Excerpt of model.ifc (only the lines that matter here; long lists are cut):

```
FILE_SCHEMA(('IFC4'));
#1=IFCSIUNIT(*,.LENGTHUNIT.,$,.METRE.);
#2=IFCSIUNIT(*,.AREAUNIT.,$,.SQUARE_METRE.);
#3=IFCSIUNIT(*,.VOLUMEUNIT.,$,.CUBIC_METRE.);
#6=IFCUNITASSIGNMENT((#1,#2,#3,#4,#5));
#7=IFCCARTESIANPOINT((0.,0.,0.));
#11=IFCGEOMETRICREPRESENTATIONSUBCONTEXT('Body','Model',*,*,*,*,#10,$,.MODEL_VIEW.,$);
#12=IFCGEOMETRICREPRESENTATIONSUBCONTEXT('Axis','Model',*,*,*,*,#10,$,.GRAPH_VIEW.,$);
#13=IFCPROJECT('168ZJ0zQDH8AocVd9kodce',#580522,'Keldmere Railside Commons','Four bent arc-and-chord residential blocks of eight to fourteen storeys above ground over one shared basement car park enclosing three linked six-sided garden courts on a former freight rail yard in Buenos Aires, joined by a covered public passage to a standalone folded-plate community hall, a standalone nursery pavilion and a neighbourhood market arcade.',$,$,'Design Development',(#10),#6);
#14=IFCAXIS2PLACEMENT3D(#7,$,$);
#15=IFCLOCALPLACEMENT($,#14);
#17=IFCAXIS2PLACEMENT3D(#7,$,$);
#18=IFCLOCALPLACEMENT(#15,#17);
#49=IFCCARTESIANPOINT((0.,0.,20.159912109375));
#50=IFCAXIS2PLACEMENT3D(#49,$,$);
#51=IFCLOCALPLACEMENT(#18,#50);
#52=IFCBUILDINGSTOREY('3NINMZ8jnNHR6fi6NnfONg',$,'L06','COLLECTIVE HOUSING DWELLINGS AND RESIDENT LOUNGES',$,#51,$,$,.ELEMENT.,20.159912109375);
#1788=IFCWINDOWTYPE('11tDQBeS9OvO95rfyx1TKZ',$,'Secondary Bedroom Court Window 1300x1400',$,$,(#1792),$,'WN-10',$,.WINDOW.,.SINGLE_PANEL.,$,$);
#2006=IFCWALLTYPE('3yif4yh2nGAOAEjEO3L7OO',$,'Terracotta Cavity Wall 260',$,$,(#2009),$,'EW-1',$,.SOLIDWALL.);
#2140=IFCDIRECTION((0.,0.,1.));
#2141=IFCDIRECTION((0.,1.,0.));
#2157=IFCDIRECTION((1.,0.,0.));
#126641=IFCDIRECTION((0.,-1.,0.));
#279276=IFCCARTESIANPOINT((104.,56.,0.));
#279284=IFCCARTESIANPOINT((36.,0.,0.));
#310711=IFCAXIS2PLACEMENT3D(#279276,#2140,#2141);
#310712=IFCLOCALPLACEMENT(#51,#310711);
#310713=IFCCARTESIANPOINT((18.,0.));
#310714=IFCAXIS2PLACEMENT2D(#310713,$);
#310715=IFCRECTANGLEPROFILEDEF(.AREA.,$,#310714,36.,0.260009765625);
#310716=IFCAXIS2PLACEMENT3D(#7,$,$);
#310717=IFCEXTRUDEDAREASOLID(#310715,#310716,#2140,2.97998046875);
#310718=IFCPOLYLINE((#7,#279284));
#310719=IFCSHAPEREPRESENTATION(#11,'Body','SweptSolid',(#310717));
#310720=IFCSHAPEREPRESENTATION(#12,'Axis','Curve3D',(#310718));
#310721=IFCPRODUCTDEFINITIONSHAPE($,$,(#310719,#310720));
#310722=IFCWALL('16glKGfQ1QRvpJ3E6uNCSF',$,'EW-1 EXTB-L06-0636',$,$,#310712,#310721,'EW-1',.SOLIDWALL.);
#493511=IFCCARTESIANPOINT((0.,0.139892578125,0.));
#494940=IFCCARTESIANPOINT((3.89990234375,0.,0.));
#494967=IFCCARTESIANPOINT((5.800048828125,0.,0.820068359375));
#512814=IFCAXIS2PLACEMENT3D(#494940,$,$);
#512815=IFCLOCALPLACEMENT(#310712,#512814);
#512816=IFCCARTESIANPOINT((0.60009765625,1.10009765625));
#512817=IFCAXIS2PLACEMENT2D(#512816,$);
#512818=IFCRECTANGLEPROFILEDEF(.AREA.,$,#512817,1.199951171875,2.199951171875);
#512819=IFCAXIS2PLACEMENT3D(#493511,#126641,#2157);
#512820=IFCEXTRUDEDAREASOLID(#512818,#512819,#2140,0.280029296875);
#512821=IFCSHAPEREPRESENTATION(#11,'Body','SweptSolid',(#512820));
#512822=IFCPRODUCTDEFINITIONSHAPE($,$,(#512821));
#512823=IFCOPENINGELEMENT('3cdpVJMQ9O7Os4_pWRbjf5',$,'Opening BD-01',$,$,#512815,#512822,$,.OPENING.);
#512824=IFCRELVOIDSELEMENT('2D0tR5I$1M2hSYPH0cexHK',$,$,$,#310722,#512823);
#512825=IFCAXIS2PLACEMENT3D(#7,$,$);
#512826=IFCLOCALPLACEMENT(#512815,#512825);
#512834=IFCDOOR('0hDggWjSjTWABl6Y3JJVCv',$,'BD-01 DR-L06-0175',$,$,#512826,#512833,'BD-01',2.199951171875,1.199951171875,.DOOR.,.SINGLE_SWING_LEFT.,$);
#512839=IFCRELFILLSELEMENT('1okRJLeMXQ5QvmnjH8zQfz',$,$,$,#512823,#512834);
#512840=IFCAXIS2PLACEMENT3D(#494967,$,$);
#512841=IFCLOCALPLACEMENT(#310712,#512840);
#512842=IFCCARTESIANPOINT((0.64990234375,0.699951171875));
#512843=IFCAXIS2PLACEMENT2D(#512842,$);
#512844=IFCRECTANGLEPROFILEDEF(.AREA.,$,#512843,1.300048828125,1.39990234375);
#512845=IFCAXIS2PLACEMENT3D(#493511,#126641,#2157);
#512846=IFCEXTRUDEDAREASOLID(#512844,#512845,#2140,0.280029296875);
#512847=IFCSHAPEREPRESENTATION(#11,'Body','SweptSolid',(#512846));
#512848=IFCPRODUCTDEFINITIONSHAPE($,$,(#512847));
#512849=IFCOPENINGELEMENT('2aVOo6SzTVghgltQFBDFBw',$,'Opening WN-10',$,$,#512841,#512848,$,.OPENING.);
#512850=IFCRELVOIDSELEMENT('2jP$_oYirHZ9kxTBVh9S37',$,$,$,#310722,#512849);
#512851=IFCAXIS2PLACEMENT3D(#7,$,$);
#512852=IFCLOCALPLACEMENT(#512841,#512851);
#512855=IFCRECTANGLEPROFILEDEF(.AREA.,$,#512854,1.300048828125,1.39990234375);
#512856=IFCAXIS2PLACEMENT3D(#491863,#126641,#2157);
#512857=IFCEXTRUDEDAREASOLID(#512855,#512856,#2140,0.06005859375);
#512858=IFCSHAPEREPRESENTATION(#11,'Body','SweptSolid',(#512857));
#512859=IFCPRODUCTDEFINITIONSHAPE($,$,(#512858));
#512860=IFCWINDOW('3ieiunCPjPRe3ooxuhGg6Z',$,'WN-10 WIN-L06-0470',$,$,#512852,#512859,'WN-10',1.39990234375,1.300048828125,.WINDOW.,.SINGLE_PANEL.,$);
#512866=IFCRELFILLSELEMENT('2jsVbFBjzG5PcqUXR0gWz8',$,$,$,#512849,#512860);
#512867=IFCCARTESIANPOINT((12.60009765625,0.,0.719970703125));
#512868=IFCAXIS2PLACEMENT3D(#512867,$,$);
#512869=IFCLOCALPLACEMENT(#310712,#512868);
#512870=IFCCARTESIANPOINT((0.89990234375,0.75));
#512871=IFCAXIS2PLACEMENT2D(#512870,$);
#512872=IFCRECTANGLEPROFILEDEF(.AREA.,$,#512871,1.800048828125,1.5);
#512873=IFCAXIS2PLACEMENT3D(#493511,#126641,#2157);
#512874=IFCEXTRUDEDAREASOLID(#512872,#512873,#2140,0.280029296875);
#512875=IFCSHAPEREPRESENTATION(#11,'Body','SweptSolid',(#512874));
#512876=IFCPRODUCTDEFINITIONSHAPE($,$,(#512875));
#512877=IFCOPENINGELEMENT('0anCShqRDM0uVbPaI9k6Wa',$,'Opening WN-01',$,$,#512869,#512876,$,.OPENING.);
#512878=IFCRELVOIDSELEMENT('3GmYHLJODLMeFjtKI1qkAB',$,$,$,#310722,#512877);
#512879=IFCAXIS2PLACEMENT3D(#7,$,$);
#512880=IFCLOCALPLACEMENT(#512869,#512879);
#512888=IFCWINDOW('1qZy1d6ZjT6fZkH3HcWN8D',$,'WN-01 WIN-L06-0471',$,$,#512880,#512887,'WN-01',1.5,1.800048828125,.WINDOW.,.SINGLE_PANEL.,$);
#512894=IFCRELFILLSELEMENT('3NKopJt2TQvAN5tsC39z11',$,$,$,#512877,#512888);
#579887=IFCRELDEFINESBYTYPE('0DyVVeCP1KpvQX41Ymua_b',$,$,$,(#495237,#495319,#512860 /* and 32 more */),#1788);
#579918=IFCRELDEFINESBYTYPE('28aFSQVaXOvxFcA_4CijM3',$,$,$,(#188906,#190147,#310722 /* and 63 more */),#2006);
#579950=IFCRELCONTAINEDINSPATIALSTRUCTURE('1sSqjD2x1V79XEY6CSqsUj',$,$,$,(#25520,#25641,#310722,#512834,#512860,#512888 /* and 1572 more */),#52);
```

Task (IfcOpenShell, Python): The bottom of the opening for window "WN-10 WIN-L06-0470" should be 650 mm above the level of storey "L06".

```python
import numpy as np
import ifcopenshell
import ifcopenshell.api.geometry
import ifcopenshell.geom
import ifcopenshell.util.element
import ifcopenshell.util.placement
import ifcopenshell.util.shape
import ifcopenshell.util.unit

model = ifcopenshell.open("model.ifc")
unit_scale = ifcopenshell.util.unit.calculate_unit_scale(model)

window = model.by_id(512860)
opening = window.FillsVoids[0].RelatingOpeningElement
storey = ifcopenshell.util.element.get_container(window, ifc_class="IfcBuildingStorey")
level = ifcopenshell.util.placement.get_local_placement(storey.ObjectPlacement)[2, 3]

# The opening's origin need not be at the sill, so measure its lowest point.
shape = ifcopenshell.geom.create_shape(ifcopenshell.geom.settings(), opening)
bottom = ifcopenshell.util.shape.get_shape_bottom_elevation(shape, shape.geometry) / unit_scale
dz = level + 0.65 - bottom

shift = np.array([0.0, 0.0, dz])
# The window is placed relative to its opening, so it follows when the opening moves.
matrix = ifcopenshell.util.placement.get_local_placement(opening.ObjectPlacement)
matrix[:3, 3] += shift
ifcopenshell.api.geometry.edit_object_placement(
    model, product=opening, matrix=matrix, is_si=False, should_transform_children=True
)

print(f"moved by {dz * unit_scale:+.3f} m")

model.write("model_edited.ifc")
```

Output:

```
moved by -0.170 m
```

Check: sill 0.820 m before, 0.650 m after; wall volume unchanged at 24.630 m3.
